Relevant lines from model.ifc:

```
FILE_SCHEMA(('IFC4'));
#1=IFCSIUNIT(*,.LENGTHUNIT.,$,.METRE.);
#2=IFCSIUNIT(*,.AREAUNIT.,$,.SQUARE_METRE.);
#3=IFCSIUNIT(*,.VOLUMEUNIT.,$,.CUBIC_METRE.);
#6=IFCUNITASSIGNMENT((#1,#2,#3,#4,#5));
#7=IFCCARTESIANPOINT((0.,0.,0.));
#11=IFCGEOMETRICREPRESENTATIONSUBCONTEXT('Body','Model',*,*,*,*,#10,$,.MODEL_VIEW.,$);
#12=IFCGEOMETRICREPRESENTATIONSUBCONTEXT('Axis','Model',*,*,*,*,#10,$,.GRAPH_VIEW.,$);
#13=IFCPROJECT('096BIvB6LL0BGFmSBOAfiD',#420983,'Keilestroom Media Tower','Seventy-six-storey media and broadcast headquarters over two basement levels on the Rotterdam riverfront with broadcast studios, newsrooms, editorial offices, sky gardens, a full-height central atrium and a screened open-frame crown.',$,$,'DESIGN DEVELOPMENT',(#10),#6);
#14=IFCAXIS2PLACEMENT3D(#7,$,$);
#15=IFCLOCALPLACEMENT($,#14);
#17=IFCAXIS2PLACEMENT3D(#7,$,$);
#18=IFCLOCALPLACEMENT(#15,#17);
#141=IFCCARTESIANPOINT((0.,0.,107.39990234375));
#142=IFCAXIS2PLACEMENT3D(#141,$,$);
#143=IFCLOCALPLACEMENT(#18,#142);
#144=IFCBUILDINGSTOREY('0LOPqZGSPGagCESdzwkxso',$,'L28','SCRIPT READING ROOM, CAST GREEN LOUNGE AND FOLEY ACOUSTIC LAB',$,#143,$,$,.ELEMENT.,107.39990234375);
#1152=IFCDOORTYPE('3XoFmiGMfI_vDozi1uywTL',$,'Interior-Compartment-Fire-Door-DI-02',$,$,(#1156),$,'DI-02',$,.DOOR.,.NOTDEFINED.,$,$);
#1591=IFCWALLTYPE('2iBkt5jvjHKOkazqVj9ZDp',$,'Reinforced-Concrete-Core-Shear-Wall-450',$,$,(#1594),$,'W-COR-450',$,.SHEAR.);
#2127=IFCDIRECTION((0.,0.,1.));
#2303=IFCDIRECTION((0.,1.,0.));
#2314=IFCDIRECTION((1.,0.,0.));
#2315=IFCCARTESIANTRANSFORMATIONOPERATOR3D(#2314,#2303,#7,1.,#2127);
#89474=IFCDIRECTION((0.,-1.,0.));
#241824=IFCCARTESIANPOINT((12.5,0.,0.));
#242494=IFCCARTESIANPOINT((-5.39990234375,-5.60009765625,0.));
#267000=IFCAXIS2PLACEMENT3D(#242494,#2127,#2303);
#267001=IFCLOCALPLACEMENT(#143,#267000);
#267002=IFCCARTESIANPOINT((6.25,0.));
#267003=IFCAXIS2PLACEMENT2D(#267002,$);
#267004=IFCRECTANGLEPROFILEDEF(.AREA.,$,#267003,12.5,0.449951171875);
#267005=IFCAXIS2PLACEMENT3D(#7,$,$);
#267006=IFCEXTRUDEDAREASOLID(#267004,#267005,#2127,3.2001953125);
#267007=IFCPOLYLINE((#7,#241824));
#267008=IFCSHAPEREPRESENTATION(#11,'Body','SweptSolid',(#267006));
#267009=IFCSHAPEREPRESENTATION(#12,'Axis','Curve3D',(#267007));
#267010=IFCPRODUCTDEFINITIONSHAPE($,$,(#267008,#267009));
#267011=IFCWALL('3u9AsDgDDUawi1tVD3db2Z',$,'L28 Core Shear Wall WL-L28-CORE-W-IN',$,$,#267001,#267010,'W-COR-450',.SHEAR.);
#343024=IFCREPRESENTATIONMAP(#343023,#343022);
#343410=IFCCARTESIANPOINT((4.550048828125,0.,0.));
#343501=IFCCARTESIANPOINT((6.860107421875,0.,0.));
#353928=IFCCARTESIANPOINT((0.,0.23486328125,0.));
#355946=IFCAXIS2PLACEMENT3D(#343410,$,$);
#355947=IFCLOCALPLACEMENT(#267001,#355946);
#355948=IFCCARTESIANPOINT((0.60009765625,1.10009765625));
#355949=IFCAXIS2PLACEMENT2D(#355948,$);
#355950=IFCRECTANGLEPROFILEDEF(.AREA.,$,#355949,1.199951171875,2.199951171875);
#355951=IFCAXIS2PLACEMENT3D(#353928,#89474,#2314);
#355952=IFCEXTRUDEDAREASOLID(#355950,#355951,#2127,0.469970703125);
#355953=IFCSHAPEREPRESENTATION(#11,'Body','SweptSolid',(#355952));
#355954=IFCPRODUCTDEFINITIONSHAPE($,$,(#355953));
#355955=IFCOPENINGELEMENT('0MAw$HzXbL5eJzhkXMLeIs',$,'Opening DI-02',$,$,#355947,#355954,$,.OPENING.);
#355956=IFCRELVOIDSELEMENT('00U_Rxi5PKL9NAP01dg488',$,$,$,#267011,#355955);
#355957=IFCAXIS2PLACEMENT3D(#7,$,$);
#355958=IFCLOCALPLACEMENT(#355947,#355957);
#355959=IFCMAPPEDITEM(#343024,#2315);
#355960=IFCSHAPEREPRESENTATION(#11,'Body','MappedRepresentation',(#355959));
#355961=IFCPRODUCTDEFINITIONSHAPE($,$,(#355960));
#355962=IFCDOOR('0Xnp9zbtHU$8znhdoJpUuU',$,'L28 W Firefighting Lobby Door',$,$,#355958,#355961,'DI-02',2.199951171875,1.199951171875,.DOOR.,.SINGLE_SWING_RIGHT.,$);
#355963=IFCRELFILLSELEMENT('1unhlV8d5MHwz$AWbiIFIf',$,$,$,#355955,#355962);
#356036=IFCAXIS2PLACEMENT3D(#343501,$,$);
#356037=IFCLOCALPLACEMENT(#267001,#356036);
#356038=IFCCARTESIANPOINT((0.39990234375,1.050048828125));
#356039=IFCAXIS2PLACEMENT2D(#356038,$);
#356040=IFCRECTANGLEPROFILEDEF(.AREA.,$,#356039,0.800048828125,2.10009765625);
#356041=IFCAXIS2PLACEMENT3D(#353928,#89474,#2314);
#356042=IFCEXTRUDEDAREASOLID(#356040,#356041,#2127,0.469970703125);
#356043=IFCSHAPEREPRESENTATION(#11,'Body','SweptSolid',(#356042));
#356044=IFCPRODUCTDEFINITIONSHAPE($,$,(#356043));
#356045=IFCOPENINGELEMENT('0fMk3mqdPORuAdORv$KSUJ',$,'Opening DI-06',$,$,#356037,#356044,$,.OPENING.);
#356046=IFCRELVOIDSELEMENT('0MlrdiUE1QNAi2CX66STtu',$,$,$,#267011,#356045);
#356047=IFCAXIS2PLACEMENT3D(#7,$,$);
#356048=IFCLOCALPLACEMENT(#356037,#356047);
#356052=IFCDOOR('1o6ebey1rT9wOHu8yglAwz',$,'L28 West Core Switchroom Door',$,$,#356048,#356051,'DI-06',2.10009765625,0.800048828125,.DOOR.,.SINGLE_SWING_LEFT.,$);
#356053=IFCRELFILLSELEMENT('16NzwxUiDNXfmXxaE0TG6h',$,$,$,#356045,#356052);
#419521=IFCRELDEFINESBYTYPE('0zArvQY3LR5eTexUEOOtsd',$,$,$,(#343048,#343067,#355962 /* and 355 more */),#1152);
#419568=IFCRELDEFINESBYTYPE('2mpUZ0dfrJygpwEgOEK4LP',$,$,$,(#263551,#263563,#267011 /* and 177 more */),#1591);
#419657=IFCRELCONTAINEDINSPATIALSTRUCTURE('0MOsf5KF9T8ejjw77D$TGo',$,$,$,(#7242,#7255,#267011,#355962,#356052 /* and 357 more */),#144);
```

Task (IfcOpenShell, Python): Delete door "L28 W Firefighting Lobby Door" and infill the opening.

```python
import ifcopenshell
import ifcopenshell.api.feature
import ifcopenshell.api.root
import ifcopenshell.geom
import ifcopenshell.util.shape

model = ifcopenshell.open("model.ifc")
settings = ifcopenshell.geom.settings()


def volume(element):
    """Net volume in cubic metres, openings subtracted."""
    shape = ifcopenshell.geom.create_shape(settings, element)
    return ifcopenshell.util.shape.get_volume(shape.geometry)


door = model.by_id(355962)
opening = door.FillsVoids[0].RelatingOpeningElement
wall = opening.VoidsElements[0].RelatingBuildingElement
before = volume(wall)

ifcopenshell.api.root.remove_product(model, product=door)
ifcopenshell.api.feature.remove_feature(model, feature=opening)

after = volume(wall)

print(f"wall volume {before:.3f} -> {after:.3f} m3")

model.write("model_updated.ifc")
```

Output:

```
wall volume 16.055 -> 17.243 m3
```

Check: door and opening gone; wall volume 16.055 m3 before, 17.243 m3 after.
